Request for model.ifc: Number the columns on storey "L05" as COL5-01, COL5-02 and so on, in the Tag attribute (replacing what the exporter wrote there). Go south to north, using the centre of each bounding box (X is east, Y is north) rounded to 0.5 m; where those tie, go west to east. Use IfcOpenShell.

First a look at what the model holds.

```python
import ifcopenshell
import ifcopenshell.util.element
import ifcopenshell.util.placement

model = ifcopenshell.open("model.ifc")
print(model.schema)
storey = next(s for s in model.by_type("IfcBuildingStorey") if s.Name == "L05")
columns = [e for e in ifcopenshell.util.element.get_decomposition(storey) if e.is_a("IfcColumn")]
for e in sorted(columns, key=lambda e: e.id()):
    origin = ifcopenshell.util.placement.get_local_placement(e.ObjectPlacement)[:3, 3]
    print(e.id(), e.Tag, e.Name, origin.round(2) + 0.0, sep=" | ")
```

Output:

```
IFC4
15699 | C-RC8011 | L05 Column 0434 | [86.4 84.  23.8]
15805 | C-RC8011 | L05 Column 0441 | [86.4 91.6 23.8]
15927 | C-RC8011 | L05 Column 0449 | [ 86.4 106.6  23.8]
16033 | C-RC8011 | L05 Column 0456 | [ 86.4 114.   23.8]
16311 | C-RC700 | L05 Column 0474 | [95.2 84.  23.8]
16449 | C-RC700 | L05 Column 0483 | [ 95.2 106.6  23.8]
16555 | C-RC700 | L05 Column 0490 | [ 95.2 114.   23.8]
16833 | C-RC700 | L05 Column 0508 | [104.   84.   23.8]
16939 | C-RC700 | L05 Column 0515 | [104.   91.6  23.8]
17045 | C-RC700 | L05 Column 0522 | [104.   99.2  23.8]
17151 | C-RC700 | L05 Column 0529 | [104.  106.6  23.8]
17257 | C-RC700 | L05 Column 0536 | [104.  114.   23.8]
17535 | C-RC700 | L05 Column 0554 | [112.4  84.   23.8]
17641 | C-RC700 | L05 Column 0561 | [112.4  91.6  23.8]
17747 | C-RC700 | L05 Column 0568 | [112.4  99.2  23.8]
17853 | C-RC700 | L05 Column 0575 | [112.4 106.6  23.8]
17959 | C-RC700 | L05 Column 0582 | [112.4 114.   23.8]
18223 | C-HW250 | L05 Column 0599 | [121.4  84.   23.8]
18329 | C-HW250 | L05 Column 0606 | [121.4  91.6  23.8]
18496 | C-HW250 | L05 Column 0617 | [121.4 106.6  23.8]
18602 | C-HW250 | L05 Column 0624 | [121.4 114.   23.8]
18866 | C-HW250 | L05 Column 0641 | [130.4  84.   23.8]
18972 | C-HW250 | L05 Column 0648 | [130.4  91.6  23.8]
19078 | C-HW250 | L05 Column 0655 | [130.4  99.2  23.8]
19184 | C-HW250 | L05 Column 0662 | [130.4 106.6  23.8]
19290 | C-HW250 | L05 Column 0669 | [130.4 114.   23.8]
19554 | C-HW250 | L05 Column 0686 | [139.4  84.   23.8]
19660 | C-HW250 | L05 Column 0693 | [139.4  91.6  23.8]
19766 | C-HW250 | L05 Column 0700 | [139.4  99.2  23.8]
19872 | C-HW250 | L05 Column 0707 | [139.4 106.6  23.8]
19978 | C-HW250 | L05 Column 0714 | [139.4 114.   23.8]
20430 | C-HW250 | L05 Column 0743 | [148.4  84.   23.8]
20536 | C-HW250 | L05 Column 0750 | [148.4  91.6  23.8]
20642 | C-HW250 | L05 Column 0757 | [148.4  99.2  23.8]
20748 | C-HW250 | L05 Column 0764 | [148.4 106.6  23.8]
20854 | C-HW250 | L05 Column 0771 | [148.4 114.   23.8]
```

```python
import ifcopenshell
import ifcopenshell.geom
import ifcopenshell.util.element
import ifcopenshell.util.shape

model = ifcopenshell.open("model.ifc")
settings = ifcopenshell.geom.settings()
settings.set("use-world-coords", True)


def centre(element):
    shape = ifcopenshell.geom.create_shape(settings, element)
    return ifcopenshell.util.shape.get_bbox_centroid(shape.geometry)


storey = next(s for s in model.by_type("IfcBuildingStorey") if s.Name == "L05")
columns = [e for e in ifcopenshell.util.element.get_decomposition(storey) if e.is_a("IfcColumn")]

# Insertion points can sit at a corner or the storey origin, so sort by the geometry (in metres).
centres = {e: centre(e) for e in columns}
columns.sort(key=lambda e: (round(centres[e][1] / 0.5), centres[e][0]))

for i, e in enumerate(columns, start=1):
    number = f"COL5-{i:02d}"
    e.Tag = number
    print(e.id(), number)

model.write("model_v2.ifc")
```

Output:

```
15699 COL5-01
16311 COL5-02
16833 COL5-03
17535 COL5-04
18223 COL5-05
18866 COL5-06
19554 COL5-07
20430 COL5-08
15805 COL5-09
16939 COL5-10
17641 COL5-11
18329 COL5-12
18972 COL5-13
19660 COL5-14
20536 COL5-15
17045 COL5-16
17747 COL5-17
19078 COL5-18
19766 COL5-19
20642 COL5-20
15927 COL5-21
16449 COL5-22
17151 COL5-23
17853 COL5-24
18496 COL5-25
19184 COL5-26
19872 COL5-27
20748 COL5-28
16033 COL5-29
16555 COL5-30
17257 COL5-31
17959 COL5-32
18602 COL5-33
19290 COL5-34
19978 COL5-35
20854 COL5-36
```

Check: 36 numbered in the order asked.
